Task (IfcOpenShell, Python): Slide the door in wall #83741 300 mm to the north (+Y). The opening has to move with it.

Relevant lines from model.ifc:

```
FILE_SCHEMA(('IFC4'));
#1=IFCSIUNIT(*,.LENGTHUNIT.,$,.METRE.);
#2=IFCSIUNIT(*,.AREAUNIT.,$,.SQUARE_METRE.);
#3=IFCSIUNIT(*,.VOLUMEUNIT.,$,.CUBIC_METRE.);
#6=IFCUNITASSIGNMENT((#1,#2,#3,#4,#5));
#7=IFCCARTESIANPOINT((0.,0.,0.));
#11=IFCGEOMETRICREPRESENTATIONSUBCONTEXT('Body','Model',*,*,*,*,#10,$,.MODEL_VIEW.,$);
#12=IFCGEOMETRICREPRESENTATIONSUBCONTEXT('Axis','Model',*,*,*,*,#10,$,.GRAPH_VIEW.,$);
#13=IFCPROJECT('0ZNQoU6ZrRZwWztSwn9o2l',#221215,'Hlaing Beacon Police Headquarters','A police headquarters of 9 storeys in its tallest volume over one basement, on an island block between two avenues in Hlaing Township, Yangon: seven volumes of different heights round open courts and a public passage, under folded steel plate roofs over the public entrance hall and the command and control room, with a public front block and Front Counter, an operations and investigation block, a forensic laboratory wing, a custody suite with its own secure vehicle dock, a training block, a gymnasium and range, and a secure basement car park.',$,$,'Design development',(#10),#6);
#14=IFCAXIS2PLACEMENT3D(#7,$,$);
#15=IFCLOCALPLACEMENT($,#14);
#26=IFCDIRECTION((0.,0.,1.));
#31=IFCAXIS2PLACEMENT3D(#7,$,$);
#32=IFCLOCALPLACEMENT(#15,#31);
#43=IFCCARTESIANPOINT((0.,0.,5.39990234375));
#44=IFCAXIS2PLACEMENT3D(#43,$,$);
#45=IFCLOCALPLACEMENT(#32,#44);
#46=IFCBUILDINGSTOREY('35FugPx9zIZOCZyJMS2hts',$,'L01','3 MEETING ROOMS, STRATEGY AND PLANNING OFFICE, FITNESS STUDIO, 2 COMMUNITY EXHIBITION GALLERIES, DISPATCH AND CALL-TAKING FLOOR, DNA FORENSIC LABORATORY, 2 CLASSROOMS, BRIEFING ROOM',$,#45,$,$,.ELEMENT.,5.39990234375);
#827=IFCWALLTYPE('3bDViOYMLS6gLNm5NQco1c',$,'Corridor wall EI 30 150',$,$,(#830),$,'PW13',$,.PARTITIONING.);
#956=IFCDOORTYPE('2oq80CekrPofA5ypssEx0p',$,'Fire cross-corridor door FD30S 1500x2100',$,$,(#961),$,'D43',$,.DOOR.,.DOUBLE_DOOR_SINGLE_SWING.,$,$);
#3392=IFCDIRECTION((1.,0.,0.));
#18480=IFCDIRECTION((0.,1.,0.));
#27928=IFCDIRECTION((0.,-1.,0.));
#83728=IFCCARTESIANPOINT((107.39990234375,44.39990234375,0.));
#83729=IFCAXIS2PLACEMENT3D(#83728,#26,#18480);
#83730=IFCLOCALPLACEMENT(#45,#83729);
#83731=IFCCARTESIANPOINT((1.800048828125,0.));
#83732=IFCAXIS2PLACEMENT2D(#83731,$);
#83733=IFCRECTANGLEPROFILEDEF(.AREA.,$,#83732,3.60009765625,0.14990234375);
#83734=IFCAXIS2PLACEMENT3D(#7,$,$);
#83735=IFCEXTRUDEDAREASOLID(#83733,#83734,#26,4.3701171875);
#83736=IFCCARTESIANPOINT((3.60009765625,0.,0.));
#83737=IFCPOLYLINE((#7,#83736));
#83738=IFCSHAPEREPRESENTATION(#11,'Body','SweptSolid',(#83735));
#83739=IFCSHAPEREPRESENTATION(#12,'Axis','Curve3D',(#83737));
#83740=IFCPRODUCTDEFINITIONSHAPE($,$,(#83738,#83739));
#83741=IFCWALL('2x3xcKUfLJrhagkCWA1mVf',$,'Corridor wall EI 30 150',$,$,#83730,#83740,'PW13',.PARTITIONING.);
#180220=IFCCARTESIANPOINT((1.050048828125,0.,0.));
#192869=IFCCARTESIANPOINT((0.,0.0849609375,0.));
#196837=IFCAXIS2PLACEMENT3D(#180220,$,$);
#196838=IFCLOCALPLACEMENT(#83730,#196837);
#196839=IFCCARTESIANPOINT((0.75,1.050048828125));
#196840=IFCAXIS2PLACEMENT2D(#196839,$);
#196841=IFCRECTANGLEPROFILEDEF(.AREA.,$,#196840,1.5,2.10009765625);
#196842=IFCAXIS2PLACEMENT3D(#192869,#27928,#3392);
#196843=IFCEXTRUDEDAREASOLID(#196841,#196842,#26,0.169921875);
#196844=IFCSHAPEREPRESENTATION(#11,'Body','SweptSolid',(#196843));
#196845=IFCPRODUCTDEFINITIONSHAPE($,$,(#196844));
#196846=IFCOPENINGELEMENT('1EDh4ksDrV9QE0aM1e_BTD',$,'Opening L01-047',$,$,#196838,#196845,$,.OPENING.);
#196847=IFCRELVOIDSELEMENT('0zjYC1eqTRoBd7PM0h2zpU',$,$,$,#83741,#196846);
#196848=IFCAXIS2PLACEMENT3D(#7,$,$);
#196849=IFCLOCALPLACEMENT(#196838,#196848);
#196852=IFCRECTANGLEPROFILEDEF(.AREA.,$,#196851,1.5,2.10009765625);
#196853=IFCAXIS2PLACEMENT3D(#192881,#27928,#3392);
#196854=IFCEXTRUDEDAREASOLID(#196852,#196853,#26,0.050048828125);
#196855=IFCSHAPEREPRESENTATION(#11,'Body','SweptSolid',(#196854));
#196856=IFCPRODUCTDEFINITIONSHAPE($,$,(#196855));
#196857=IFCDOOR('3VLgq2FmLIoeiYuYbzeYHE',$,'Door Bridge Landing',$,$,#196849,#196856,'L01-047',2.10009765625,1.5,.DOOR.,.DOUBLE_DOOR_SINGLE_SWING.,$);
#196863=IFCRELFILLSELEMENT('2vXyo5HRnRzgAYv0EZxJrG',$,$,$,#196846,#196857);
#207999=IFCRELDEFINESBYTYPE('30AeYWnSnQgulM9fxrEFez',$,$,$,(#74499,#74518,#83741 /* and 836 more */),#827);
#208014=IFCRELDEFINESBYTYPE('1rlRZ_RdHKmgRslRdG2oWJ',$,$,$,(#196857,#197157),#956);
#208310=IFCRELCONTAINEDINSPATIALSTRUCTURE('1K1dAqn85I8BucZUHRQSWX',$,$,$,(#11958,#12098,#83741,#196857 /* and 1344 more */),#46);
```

```python
import ifcopenshell
import ifcopenshell.api.geometry
import ifcopenshell.util.placement

model = ifcopenshell.open("model.ifc")

door = model.by_guid("3VLgq2FmLIoeiYuYbzeYHE")
opening = door.FillsVoids[0].RelatingOpeningElement
wall = opening.VoidsElements[0].RelatingBuildingElement

wall_matrix = ifcopenshell.util.placement.get_local_placement(wall.ObjectPlacement)
shift = wall_matrix[:3, 0] * 0.3
before = ifcopenshell.util.placement.get_local_placement(door.ObjectPlacement)[:3, 3].copy()

# The door is placed relative to its opening, so it follows when the opening moves.
matrix = ifcopenshell.util.placement.get_local_placement(opening.ObjectPlacement)
matrix[:3, 3] += shift
ifcopenshell.api.geometry.edit_object_placement(
    model, product=opening, matrix=matrix, is_si=False, should_transform_children=True
)

after = ifcopenshell.util.placement.get_local_placement(door.ObjectPlacement)[:3, 3]
print("door moved by", (after - before).round(3) + 0.0)

model.write("model_v2.ifc")
```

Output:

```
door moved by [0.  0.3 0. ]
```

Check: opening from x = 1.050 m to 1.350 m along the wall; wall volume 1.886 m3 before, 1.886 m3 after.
